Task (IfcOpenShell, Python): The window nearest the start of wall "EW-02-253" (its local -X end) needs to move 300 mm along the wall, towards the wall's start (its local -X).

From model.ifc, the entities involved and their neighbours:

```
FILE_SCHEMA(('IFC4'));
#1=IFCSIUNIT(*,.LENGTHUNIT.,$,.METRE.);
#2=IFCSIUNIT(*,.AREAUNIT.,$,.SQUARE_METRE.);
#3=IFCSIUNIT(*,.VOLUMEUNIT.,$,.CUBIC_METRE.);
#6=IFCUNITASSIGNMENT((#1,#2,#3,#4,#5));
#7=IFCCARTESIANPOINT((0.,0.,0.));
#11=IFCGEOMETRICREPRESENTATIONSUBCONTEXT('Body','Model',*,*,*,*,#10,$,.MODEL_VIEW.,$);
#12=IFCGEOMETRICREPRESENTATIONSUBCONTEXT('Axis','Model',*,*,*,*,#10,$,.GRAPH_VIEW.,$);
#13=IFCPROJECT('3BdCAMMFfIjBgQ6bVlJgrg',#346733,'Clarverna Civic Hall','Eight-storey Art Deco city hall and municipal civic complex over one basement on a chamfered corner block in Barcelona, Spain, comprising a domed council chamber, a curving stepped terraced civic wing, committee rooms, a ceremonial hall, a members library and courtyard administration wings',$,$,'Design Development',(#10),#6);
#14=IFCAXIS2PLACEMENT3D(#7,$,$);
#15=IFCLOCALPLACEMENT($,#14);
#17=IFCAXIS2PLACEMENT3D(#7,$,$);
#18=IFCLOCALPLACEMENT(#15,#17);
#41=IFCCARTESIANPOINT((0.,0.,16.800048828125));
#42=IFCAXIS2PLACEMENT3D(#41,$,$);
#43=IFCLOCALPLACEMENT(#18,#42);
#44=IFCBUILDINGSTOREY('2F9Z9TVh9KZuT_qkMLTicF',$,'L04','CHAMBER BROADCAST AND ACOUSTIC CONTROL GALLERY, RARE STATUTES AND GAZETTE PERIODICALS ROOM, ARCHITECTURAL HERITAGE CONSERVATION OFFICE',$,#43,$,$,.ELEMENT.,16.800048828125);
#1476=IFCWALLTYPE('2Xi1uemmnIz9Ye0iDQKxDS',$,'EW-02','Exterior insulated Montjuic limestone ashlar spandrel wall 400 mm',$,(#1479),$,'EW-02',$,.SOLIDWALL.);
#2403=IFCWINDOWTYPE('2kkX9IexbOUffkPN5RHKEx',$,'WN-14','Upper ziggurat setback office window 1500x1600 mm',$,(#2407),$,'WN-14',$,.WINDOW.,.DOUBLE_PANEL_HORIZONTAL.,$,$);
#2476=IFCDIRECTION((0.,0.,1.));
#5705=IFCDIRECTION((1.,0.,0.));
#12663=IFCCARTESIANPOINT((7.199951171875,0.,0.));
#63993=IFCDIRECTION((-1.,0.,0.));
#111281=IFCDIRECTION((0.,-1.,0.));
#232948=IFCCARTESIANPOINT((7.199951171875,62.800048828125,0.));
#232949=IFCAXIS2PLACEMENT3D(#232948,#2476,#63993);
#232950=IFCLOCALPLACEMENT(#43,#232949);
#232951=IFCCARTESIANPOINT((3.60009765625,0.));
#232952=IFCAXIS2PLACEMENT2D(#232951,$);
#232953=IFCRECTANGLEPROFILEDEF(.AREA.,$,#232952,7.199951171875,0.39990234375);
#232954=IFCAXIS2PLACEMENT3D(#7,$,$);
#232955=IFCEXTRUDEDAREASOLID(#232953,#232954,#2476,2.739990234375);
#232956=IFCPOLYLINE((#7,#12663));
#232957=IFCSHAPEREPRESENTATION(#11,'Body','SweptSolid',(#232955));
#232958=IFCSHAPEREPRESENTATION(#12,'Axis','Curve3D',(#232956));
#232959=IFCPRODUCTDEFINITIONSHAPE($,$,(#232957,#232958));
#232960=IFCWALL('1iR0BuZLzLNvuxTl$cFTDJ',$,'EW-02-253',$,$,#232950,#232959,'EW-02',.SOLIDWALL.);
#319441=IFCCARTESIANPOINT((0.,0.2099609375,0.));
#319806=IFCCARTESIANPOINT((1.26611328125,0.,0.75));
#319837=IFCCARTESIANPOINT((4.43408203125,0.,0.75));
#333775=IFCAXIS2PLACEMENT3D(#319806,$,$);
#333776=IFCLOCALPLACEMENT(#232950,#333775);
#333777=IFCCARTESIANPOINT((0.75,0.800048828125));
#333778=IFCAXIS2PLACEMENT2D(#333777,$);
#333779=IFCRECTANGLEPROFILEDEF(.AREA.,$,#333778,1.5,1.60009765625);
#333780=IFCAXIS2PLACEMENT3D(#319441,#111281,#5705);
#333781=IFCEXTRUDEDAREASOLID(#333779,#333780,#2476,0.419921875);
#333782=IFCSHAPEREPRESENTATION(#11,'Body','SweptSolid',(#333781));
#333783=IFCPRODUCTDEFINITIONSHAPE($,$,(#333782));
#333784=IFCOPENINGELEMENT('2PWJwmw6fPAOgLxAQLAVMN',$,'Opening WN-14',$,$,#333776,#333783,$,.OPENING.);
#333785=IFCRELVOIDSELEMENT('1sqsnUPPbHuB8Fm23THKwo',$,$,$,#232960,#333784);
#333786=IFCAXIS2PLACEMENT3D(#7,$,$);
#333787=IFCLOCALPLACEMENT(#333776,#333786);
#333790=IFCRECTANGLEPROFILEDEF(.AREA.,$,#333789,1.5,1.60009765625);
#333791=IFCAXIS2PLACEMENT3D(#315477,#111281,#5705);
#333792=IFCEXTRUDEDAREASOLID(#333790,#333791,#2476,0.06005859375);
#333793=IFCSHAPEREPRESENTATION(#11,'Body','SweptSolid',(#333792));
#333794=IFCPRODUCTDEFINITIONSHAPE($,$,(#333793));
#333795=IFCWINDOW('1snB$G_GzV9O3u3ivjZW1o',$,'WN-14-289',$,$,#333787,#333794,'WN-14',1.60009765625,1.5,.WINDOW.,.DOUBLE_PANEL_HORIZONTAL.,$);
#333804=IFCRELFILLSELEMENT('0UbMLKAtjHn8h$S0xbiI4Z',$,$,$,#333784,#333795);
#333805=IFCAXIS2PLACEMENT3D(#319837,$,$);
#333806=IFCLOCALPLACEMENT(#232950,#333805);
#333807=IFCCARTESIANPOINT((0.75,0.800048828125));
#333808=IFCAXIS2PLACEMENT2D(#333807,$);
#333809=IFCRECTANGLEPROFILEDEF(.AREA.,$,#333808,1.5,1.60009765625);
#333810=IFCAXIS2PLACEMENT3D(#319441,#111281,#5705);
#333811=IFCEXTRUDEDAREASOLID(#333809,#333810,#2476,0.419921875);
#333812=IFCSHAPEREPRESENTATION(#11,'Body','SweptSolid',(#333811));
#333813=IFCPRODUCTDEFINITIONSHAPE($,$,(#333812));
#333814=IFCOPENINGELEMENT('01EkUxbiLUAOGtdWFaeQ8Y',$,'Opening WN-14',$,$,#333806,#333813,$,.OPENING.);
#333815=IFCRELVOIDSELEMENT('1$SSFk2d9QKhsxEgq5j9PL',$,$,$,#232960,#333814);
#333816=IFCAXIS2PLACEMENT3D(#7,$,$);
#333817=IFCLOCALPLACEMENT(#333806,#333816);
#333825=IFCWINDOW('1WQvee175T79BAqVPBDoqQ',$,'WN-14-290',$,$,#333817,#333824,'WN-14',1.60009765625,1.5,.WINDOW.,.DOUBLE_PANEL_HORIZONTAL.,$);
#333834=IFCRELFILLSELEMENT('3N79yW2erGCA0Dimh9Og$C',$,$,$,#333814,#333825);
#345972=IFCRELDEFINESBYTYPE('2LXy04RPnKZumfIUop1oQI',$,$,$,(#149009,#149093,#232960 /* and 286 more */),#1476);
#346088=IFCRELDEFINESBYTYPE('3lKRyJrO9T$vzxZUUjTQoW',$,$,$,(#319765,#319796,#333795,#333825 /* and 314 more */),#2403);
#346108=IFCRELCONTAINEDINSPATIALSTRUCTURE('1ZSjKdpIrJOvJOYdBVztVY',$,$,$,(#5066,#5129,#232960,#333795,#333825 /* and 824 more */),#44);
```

```python
import ifcopenshell
import ifcopenshell.api.geometry
import ifcopenshell.util.placement
import ifcopenshell.util.unit

model = ifcopenshell.open("model.ifc")
unit_scale = ifcopenshell.util.unit.calculate_unit_scale(model)

window = model.by_guid("1snB$G_GzV9O3u3ivjZW1o")
opening = window.FillsVoids[0].RelatingOpeningElement
wall = opening.VoidsElements[0].RelatingBuildingElement

wall_matrix = ifcopenshell.util.placement.get_local_placement(wall.ObjectPlacement)
shift = wall_matrix[:3, 0] * -0.3 / unit_scale
before = ifcopenshell.util.placement.get_local_placement(window.ObjectPlacement)[:3, 3].copy()

# The window is placed relative to its opening, so it follows when the opening moves.
matrix = ifcopenshell.util.placement.get_local_placement(opening.ObjectPlacement)
matrix[:3, 3] += shift
ifcopenshell.api.geometry.edit_object_placement(
    model, product=opening, matrix=matrix, is_si=False, should_transform_children=True
)

after = ifcopenshell.util.placement.get_local_placement(window.ObjectPlacement)[:3, 3]
print("window moved by", (after - before).round(3) + 0.0)

model.write("model_updated.ifc")
```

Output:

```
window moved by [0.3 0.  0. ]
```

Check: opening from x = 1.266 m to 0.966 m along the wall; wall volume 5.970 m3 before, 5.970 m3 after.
